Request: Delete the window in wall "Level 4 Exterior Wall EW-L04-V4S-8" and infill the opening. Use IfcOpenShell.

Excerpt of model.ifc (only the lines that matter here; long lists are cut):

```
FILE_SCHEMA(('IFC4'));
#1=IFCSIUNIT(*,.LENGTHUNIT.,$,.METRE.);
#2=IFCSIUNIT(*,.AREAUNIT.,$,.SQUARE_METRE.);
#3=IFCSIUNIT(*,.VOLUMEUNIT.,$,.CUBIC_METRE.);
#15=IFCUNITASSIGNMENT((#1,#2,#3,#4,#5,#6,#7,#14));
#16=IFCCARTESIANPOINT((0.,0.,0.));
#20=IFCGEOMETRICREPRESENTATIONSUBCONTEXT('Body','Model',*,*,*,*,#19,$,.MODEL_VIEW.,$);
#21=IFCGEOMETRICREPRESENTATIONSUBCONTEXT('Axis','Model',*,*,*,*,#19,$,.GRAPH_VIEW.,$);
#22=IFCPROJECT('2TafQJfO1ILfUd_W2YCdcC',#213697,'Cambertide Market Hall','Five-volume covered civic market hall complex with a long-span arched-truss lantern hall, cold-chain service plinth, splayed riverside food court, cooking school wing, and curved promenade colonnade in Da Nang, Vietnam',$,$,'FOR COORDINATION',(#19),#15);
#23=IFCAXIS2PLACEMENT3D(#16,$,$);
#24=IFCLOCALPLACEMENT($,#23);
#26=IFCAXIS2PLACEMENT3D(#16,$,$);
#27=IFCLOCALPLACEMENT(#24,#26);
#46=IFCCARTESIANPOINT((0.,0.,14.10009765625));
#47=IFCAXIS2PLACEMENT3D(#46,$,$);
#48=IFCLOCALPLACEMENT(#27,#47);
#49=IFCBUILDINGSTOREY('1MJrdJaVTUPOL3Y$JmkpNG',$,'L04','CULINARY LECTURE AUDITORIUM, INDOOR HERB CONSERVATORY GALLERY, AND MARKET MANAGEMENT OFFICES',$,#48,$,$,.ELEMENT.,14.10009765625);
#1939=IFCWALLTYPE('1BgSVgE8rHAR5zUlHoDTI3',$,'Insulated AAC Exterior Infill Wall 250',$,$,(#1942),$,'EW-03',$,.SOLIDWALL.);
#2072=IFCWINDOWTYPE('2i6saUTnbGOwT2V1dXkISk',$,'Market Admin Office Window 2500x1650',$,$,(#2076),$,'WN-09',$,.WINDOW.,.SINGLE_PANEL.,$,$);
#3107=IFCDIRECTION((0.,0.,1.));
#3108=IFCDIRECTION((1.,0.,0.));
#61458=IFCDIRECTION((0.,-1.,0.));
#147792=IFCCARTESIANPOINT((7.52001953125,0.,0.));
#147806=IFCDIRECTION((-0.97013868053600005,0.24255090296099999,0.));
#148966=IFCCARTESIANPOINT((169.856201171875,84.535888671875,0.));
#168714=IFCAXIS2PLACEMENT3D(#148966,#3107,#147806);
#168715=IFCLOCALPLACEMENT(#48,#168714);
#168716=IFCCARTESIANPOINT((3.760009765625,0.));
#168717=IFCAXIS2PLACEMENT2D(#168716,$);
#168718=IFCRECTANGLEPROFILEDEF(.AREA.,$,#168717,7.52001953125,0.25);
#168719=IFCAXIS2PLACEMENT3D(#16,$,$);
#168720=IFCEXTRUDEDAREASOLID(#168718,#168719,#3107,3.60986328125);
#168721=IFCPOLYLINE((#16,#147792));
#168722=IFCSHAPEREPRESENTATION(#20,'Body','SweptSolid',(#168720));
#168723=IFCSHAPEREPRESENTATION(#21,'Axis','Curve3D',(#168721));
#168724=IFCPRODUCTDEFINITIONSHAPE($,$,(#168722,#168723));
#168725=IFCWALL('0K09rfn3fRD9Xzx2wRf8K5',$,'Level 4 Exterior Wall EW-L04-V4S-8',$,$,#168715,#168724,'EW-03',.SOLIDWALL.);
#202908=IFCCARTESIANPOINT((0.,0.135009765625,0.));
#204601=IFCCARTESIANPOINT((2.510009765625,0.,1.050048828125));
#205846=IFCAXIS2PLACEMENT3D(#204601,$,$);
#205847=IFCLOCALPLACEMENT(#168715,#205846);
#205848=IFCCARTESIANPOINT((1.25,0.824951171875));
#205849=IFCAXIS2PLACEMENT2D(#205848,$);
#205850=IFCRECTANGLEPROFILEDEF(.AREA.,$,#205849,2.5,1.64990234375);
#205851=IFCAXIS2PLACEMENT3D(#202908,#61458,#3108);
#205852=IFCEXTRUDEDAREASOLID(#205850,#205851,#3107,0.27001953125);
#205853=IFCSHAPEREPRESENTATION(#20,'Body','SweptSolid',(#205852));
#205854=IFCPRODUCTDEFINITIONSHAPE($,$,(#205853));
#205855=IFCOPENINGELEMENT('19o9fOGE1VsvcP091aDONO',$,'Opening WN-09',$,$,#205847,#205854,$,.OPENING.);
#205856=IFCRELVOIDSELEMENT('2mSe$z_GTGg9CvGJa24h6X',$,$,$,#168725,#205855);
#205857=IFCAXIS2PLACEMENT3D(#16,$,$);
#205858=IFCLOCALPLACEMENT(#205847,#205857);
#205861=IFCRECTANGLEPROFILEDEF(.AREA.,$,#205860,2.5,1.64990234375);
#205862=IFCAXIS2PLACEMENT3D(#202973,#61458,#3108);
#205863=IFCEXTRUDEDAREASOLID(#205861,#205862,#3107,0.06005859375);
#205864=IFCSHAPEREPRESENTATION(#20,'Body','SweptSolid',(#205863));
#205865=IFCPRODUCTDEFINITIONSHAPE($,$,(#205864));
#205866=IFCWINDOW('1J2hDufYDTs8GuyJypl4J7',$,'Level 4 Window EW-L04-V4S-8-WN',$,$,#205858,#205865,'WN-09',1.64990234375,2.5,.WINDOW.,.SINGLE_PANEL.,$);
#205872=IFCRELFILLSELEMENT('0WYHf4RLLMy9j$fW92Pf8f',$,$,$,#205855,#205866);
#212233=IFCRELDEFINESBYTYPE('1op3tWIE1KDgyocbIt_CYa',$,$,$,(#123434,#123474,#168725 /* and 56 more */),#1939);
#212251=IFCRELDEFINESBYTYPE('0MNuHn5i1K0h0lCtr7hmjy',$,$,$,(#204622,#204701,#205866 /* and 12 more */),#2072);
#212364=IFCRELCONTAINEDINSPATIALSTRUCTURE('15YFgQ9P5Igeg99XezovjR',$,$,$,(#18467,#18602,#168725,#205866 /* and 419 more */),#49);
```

```python
import ifcopenshell
import ifcopenshell.api.feature
import ifcopenshell.api.root
import ifcopenshell.geom
import ifcopenshell.util.shape

model = ifcopenshell.open("model.ifc")
settings = ifcopenshell.geom.settings()


def volume(element):
    """Net volume in cubic metres, openings subtracted."""
    shape = ifcopenshell.geom.create_shape(settings, element)
    return ifcopenshell.util.shape.get_volume(shape.geometry)


window = model.by_guid("1J2hDufYDTs8GuyJypl4J7")
opening = window.FillsVoids[0].RelatingOpeningElement
wall = opening.VoidsElements[0].RelatingBuildingElement
before = volume(wall)

ifcopenshell.api.root.remove_product(model, product=window)
ifcopenshell.api.feature.remove_feature(model, feature=opening)

after = volume(wall)

print(f"wall volume {before:.3f} -> {after:.3f} m3")

model.write("model_v2.ifc")
```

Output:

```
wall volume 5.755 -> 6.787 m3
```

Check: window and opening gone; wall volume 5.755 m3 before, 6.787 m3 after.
